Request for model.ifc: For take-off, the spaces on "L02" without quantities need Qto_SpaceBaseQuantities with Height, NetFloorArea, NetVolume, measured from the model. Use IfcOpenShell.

First a look at what the model holds.

```python
import ifcopenshell
import ifcopenshell.util.element
import ifcopenshell.util.unit

model = ifcopenshell.open("model.ifc")
print(model.schema)
for unit_type in ("LENGTHUNIT", "AREAUNIT", "VOLUMEUNIT"):
    print(unit_type, ifcopenshell.util.unit.calculate_unit_scale(model, unit_type))
storey = next(s for s in model.by_type("IfcBuildingStorey") if s.Name == "L02")
spaces = [e for e in ifcopenshell.util.element.get_decomposition(storey) if e.is_a("IfcSpace")]
for e in sorted(spaces, key=lambda e: e.id()):
    print(e.id(), e.is_a(), e.Name, list(ifcopenshell.util.element.get_psets(e, qtos_only=True)), sep=" | ")
```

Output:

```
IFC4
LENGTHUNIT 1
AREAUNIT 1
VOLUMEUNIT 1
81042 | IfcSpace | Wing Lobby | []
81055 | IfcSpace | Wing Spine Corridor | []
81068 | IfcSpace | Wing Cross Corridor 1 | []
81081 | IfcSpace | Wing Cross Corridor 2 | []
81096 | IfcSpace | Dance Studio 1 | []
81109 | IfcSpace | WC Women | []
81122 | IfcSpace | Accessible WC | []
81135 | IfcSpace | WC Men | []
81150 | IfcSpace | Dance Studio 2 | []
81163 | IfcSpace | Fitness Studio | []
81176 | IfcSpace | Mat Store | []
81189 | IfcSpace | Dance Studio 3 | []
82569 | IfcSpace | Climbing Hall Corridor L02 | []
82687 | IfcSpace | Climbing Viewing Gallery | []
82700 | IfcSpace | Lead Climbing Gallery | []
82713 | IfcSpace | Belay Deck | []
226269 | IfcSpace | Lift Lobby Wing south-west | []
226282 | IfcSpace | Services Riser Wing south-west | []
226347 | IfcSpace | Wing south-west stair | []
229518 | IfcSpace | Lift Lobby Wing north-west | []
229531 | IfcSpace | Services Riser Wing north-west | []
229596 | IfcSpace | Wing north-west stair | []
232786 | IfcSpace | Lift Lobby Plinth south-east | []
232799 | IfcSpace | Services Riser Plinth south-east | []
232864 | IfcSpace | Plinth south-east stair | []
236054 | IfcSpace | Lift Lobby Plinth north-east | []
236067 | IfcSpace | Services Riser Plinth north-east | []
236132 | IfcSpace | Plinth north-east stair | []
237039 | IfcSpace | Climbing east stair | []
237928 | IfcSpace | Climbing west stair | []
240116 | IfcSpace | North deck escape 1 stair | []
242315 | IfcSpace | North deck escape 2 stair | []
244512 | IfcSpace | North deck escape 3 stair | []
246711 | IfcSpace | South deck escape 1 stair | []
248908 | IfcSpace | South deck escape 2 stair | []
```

```python
import ifcopenshell
import ifcopenshell.api.pset
import ifcopenshell.geom
import ifcopenshell.util.element
import ifcopenshell.util.shape
import ifcopenshell.util.unit

model = ifcopenshell.open("model.ifc")
unit_scale = ifcopenshell.util.unit.calculate_unit_scale(model)
area_scale = ifcopenshell.util.unit.calculate_unit_scale(model, "AREAUNIT")
volume_scale = ifcopenshell.util.unit.calculate_unit_scale(model, "VOLUMEUNIT")
settings = ifcopenshell.geom.settings()

storey = next(s for s in model.by_type("IfcBuildingStorey") if s.Name == "L02")
spaces = [e for e in ifcopenshell.util.element.get_decomposition(storey) if e.is_a("IfcSpace")]

for e in sorted(spaces, key=lambda e: e.id()):
    if ifcopenshell.util.element.get_psets(e, qtos_only=True, should_inherit=False):
        continue
    # Geometry comes back in metres, in the element's own axes.
    shape = ifcopenshell.geom.create_shape(settings, e)
    values = {
        "Height": ifcopenshell.util.shape.get_z(shape.geometry) / unit_scale,
        "NetFloorArea": ifcopenshell.util.shape.get_footprint_area(shape.geometry) / area_scale,
        "NetVolume": ifcopenshell.util.shape.get_volume(shape.geometry) / volume_scale,
    }
    qto = ifcopenshell.api.pset.add_qto(model, product=e, name="Qto_SpaceBaseQuantities")
    ifcopenshell.api.pset.edit_qto(model, qto=qto, properties=values)
    print(e.id(), {k: round(v, 3) for k, v in values.items()})

model.write("model_rev.ifc")
```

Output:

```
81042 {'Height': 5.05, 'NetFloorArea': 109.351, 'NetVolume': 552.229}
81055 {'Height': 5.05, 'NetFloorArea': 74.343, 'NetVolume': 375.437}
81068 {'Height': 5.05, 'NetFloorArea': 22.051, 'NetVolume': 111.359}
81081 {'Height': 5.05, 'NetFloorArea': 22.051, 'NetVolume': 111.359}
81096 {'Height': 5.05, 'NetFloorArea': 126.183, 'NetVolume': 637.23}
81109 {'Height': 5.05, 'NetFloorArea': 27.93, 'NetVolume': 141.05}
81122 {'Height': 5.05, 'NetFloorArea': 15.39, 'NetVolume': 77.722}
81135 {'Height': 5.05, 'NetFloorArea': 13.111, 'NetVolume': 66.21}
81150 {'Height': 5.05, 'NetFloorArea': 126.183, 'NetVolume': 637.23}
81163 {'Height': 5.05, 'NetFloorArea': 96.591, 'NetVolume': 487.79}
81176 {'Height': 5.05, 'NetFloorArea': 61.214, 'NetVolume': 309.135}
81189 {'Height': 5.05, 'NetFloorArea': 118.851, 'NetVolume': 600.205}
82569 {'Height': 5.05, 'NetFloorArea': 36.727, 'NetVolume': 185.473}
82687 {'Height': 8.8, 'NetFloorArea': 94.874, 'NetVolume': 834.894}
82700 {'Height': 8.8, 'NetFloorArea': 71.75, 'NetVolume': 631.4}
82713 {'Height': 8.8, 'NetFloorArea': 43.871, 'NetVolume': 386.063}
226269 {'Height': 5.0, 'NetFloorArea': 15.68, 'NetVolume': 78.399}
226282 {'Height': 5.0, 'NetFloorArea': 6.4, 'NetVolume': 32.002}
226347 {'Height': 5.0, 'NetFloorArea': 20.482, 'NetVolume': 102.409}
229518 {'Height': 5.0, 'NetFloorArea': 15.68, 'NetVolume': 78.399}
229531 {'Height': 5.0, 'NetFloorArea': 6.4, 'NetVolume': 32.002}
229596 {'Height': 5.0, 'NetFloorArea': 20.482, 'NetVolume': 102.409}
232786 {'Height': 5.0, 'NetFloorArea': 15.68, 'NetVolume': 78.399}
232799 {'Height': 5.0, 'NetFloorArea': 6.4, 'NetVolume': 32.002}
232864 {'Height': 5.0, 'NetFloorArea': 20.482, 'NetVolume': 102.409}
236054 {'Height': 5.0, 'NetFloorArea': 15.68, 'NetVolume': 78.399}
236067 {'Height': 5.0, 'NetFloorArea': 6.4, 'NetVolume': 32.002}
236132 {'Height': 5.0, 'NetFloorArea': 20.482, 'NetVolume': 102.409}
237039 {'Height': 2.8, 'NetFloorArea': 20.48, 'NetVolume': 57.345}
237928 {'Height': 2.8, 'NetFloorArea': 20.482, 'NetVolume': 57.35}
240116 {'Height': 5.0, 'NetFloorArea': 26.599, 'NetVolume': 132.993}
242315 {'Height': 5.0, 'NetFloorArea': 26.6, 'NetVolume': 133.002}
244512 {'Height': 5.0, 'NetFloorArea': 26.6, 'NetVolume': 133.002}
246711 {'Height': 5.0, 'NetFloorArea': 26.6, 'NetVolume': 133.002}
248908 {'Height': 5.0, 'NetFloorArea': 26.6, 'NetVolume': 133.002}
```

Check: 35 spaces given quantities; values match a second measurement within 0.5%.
